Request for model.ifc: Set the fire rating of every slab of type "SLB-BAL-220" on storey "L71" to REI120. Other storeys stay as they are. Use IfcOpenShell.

First a look at what the model holds.

```python
import ifcopenshell
import ifcopenshell.util.element

model = ifcopenshell.open("model.ifc")
print(model.schema)
storey = next(s for s in model.by_type("IfcBuildingStorey") if s.Name == "L71")
slabs = [e for e in ifcopenshell.util.element.get_decomposition(storey) if e.is_a("IfcSlab")]
seen = {}
for e in slabs:
    element_type = ifcopenshell.util.element.get_type(e)
    key = (element_type.Name if element_type != e and element_type else None, ifcopenshell.util.element.get_pset(e, "Pset_SlabCommon", "FireRating"))
    seen[key] = seen.get(key, 0) + 1
for (name, value), count in sorted(seen.items(), key=str):
    print(count, "x", name, "|", value)
```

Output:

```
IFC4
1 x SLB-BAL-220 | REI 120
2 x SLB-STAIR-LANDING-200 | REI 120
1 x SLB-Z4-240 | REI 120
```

```python
import ifcopenshell
import ifcopenshell.api.pset
import ifcopenshell.util.element

model = ifcopenshell.open("model.ifc")

storey = next(s for s in model.by_type("IfcBuildingStorey") if s.Name == "L71")
slabs = [e for e in ifcopenshell.util.element.get_decomposition(storey) if e.is_a("IfcSlab")]

count = 0
for e in slabs:
    element_type = ifcopenshell.util.element.get_type(e)
    if element_type in (None, e) or element_type.Name != "SLB-BAL-220":
        continue
    found = ifcopenshell.util.element.get_pset(e, "Pset_SlabCommon", should_inherit=False)
    if found:
        pset = model.by_id(found["id"])
        if len(ifcopenshell.util.element.get_elements_by_pset(pset)) > 1:
            pset = ifcopenshell.api.pset.unshare_pset(model, products=[e], pset=pset)[0]
    else:
        pset = ifcopenshell.api.pset.add_pset(model, product=e, name="Pset_SlabCommon")
    ifcopenshell.api.pset.edit_pset(model, pset=pset, properties={"FireRating": "REI120"})
    count += 1

print(count, "slabs updated")

model.write("model_v2.ifc")
```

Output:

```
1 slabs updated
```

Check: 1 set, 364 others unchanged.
